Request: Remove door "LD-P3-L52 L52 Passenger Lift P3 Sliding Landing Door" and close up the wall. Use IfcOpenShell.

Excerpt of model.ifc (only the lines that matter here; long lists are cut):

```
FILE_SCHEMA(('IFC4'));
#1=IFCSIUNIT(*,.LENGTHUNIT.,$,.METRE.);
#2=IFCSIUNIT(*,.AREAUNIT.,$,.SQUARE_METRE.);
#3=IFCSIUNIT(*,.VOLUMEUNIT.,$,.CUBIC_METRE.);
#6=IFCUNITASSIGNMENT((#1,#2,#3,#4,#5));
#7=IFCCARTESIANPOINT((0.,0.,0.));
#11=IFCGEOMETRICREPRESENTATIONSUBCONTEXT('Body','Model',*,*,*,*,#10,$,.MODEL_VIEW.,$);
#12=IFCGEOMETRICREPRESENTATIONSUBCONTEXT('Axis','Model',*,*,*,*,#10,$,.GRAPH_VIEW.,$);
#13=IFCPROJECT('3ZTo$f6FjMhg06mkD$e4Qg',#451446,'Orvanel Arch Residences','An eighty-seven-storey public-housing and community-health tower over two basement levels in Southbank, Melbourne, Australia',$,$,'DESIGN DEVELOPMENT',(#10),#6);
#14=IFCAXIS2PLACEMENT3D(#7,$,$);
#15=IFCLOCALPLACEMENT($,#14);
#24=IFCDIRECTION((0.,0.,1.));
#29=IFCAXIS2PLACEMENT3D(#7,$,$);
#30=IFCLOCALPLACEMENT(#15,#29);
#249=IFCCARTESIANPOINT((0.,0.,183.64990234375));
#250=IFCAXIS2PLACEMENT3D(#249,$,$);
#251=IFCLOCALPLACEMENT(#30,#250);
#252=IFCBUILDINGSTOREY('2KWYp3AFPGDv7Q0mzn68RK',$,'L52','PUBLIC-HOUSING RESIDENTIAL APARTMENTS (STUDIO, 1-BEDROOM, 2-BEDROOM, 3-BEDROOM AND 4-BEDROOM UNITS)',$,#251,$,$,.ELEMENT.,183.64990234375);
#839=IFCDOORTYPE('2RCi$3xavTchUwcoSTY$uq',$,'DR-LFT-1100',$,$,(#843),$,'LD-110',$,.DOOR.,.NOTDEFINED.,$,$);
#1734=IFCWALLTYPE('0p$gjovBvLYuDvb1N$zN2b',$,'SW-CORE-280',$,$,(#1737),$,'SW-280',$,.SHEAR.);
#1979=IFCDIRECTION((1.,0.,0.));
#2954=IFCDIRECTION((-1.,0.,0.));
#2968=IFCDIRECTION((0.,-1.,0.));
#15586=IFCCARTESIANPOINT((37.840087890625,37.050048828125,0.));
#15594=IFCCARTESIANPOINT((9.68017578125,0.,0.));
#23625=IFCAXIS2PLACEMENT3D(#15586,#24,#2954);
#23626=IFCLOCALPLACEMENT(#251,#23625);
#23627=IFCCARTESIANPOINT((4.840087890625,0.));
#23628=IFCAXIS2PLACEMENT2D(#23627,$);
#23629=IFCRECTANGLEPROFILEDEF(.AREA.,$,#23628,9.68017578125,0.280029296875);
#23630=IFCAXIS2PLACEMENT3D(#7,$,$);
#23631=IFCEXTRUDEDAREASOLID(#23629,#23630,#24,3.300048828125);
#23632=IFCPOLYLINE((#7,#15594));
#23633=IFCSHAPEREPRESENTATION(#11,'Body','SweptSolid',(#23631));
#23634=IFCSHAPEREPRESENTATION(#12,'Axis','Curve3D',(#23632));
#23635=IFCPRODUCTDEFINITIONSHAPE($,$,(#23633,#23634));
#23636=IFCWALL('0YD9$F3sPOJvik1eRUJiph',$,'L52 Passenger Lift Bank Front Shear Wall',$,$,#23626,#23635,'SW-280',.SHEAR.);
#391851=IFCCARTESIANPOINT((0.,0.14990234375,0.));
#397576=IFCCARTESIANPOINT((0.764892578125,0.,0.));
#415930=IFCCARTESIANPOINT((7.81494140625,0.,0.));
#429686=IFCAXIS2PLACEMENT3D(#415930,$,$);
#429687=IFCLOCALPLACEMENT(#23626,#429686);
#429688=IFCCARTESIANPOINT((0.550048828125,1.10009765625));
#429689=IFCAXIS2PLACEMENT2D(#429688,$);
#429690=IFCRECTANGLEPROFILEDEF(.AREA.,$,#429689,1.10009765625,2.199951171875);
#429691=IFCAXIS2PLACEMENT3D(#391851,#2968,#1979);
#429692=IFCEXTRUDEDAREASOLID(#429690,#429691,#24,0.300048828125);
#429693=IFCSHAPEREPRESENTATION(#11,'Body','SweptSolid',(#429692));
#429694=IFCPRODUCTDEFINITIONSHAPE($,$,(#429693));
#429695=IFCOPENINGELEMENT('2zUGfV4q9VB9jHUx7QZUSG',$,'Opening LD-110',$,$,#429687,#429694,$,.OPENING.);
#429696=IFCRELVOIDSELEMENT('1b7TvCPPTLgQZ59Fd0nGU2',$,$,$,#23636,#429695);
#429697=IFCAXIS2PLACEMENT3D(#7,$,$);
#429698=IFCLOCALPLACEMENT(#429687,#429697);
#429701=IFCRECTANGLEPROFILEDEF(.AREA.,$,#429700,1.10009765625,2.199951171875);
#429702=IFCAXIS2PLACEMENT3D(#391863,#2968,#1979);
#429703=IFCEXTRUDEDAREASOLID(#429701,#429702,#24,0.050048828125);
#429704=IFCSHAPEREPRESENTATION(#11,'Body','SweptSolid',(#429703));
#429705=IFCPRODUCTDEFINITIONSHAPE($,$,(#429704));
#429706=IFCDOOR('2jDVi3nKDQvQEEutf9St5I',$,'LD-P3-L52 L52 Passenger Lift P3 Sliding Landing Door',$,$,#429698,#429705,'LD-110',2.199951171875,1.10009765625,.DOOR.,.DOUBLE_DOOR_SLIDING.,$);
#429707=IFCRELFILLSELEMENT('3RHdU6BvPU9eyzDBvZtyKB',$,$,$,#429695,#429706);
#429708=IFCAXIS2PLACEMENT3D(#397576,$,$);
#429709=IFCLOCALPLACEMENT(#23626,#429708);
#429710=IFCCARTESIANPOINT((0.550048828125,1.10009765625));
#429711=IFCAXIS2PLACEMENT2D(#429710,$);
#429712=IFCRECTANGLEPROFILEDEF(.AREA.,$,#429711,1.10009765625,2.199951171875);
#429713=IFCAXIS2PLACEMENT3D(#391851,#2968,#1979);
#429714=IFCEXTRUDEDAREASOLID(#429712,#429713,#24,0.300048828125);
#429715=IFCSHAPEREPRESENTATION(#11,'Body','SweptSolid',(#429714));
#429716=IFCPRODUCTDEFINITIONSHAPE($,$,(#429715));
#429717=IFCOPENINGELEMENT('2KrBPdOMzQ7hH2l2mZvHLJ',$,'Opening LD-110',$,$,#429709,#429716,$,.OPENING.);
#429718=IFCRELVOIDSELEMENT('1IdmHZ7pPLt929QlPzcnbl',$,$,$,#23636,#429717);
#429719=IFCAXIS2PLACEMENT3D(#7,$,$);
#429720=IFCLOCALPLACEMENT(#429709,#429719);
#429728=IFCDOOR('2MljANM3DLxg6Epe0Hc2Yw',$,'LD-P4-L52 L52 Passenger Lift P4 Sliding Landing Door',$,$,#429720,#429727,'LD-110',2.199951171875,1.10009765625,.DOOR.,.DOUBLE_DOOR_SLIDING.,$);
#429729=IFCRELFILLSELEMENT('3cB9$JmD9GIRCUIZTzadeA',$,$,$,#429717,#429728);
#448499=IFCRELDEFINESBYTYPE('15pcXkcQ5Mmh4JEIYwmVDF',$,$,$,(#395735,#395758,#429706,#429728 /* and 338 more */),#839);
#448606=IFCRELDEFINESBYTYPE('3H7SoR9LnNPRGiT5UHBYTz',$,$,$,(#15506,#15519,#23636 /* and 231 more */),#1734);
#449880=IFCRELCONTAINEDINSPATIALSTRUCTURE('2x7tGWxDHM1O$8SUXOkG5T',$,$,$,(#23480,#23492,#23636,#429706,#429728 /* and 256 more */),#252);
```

```python
import ifcopenshell
import ifcopenshell.api.feature
import ifcopenshell.api.root
import ifcopenshell.geom
import ifcopenshell.util.shape

model = ifcopenshell.open("model.ifc")
settings = ifcopenshell.geom.settings()


def volume(element):
    """Net volume in cubic metres, openings subtracted."""
    shape = ifcopenshell.geom.create_shape(settings, element)
    return ifcopenshell.util.shape.get_volume(shape.geometry)


door = model.by_guid("2jDVi3nKDQvQEEutf9St5I")
opening = door.FillsVoids[0].RelatingOpeningElement
wall = opening.VoidsElements[0].RelatingBuildingElement
before = volume(wall)

ifcopenshell.api.root.remove_product(model, product=door)
ifcopenshell.api.feature.remove_feature(model, feature=opening)

after = volume(wall)

print(f"wall volume {before:.3f} -> {after:.3f} m3")

model.write("model-out.ifc")
```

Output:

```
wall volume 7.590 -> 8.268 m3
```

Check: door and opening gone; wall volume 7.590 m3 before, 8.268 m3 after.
